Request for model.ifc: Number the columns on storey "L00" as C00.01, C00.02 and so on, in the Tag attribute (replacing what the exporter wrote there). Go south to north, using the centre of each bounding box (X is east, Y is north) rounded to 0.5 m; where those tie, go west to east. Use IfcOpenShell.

First a look at what the model holds.

```python
import ifcopenshell
import ifcopenshell.util.element
import ifcopenshell.util.placement

model = ifcopenshell.open("model.ifc")
print(model.schema)
storey = next(s for s in model.by_type("IfcBuildingStorey") if s.Name == "L00")
columns = [e for e in ifcopenshell.util.element.get_decomposition(storey) if e.is_a("IfcColumn")]
for e in sorted(columns, key=lambda e: e.id()):
    origin = ifcopenshell.util.placement.get_local_placement(e.ObjectPlacement)[:3, 3]
    print(e.id(), e.Tag, e.Name, origin.round(2) + 0.0, sep=" | ")
```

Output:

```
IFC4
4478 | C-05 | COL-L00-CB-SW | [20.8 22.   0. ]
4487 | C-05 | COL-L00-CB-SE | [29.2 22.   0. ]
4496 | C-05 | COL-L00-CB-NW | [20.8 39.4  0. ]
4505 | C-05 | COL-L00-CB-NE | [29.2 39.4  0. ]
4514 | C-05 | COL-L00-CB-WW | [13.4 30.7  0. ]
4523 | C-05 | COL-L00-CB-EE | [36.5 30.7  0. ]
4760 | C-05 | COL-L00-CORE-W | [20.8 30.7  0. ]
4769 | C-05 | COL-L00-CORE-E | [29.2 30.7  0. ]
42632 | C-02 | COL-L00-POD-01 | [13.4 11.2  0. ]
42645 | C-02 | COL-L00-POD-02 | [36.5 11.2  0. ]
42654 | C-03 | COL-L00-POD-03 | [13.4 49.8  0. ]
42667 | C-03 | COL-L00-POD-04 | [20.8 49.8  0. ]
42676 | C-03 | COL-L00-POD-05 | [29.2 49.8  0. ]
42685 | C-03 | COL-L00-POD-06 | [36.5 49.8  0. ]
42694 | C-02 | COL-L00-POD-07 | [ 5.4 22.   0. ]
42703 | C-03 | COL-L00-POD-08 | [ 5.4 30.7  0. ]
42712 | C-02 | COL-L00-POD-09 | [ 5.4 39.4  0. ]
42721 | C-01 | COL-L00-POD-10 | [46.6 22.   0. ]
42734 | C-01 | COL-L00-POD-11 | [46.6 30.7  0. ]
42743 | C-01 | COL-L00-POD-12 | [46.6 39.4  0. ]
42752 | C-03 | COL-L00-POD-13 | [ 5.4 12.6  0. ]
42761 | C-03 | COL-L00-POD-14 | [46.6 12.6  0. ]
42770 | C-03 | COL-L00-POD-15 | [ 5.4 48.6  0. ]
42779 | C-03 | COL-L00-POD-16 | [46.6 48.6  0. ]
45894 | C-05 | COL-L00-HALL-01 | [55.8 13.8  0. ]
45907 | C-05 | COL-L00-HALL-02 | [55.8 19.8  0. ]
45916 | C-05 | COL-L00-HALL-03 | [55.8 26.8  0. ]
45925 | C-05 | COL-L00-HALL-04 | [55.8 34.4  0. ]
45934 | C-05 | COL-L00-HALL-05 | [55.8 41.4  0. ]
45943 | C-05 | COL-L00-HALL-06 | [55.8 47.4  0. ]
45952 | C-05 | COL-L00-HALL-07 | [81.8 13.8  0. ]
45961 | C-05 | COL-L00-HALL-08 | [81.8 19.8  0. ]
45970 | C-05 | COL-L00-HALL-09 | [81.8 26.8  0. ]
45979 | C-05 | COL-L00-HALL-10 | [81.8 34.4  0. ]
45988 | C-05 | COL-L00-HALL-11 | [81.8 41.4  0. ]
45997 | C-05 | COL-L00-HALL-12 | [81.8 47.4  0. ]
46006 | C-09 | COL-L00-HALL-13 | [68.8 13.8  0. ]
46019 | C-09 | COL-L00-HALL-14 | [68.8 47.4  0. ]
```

```python
import ifcopenshell
import ifcopenshell.geom
import ifcopenshell.util.element
import ifcopenshell.util.shape

model = ifcopenshell.open("model.ifc")
settings = ifcopenshell.geom.settings()
settings.set("use-world-coords", True)


def centre(element):
    shape = ifcopenshell.geom.create_shape(settings, element)
    return ifcopenshell.util.shape.get_bbox_centroid(shape.geometry)


storey = next(s for s in model.by_type("IfcBuildingStorey") if s.Name == "L00")
columns = [e for e in ifcopenshell.util.element.get_decomposition(storey) if e.is_a("IfcColumn")]

# Insertion points can sit at a corner or the storey origin, so sort by the geometry (in metres).
centres = {e: centre(e) for e in columns}
columns.sort(key=lambda e: (round(centres[e][1] / 0.5), centres[e][0]))

for i, e in enumerate(columns, start=1):
    number = f"C00.{i:02d}"
    e.Tag = number
    print(e.id(), number)

model.write("model_updated.ifc")
```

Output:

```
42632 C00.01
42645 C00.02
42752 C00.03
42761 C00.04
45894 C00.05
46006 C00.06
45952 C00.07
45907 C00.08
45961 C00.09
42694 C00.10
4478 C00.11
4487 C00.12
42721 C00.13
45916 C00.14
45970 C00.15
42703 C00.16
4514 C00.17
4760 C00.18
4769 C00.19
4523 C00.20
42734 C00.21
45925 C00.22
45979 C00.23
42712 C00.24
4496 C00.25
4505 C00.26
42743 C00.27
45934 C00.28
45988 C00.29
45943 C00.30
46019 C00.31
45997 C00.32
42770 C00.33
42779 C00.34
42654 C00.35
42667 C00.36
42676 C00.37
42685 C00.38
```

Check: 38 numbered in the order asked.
